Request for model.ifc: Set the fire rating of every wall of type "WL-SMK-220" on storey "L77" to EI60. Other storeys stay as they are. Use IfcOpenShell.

First a look at what the model holds.

```python
import ifcopenshell
import ifcopenshell.util.element

model = ifcopenshell.open("model.ifc")
print(model.schema)
storey = next(s for s in model.by_type("IfcBuildingStorey") if s.Name == "L77")
walls = [e for e in ifcopenshell.util.element.get_decomposition(storey) if e.is_a("IfcWall")]
seen = {}
for e in walls:
    element_type = ifcopenshell.util.element.get_type(e)
    key = (element_type.Name if element_type != e and element_type else None, ifcopenshell.util.element.get_pset(e, "Pset_WallCommon", "FireRating"))
    seen[key] = seen.get(key, 0) + 1
for (name, value), count in sorted(seen.items(), key=str):
    print(count, "x", name, "|", value)
```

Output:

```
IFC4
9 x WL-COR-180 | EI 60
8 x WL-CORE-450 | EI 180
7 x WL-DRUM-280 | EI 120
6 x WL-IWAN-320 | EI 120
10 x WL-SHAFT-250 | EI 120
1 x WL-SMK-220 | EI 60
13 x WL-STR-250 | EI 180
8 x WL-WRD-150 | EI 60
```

```python
import ifcopenshell
import ifcopenshell.api.pset
import ifcopenshell.util.element

model = ifcopenshell.open("model.ifc")

storey = next(s for s in model.by_type("IfcBuildingStorey") if s.Name == "L77")
walls = [e for e in ifcopenshell.util.element.get_decomposition(storey) if e.is_a("IfcWall")]

count = 0
for e in walls:
    element_type = ifcopenshell.util.element.get_type(e)
    if element_type in (None, e) or element_type.Name != "WL-SMK-220":
        continue
    found = ifcopenshell.util.element.get_pset(e, "Pset_WallCommon", should_inherit=False)
    if found:
        pset = model.by_id(found["id"])
        if len(ifcopenshell.util.element.get_elements_by_pset(pset)) > 1:
            pset = ifcopenshell.api.pset.unshare_pset(model, products=[e], pset=pset)[0]
    else:
        pset = ifcopenshell.api.pset.add_pset(model, product=e, name="Pset_WallCommon")
    ifcopenshell.api.pset.edit_pset(model, pset=pset, properties={"FireRating": "EI60"})
    count += 1

print(count, "walls updated")

model.write("model_rev.ifc")
```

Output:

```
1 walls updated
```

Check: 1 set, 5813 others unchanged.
